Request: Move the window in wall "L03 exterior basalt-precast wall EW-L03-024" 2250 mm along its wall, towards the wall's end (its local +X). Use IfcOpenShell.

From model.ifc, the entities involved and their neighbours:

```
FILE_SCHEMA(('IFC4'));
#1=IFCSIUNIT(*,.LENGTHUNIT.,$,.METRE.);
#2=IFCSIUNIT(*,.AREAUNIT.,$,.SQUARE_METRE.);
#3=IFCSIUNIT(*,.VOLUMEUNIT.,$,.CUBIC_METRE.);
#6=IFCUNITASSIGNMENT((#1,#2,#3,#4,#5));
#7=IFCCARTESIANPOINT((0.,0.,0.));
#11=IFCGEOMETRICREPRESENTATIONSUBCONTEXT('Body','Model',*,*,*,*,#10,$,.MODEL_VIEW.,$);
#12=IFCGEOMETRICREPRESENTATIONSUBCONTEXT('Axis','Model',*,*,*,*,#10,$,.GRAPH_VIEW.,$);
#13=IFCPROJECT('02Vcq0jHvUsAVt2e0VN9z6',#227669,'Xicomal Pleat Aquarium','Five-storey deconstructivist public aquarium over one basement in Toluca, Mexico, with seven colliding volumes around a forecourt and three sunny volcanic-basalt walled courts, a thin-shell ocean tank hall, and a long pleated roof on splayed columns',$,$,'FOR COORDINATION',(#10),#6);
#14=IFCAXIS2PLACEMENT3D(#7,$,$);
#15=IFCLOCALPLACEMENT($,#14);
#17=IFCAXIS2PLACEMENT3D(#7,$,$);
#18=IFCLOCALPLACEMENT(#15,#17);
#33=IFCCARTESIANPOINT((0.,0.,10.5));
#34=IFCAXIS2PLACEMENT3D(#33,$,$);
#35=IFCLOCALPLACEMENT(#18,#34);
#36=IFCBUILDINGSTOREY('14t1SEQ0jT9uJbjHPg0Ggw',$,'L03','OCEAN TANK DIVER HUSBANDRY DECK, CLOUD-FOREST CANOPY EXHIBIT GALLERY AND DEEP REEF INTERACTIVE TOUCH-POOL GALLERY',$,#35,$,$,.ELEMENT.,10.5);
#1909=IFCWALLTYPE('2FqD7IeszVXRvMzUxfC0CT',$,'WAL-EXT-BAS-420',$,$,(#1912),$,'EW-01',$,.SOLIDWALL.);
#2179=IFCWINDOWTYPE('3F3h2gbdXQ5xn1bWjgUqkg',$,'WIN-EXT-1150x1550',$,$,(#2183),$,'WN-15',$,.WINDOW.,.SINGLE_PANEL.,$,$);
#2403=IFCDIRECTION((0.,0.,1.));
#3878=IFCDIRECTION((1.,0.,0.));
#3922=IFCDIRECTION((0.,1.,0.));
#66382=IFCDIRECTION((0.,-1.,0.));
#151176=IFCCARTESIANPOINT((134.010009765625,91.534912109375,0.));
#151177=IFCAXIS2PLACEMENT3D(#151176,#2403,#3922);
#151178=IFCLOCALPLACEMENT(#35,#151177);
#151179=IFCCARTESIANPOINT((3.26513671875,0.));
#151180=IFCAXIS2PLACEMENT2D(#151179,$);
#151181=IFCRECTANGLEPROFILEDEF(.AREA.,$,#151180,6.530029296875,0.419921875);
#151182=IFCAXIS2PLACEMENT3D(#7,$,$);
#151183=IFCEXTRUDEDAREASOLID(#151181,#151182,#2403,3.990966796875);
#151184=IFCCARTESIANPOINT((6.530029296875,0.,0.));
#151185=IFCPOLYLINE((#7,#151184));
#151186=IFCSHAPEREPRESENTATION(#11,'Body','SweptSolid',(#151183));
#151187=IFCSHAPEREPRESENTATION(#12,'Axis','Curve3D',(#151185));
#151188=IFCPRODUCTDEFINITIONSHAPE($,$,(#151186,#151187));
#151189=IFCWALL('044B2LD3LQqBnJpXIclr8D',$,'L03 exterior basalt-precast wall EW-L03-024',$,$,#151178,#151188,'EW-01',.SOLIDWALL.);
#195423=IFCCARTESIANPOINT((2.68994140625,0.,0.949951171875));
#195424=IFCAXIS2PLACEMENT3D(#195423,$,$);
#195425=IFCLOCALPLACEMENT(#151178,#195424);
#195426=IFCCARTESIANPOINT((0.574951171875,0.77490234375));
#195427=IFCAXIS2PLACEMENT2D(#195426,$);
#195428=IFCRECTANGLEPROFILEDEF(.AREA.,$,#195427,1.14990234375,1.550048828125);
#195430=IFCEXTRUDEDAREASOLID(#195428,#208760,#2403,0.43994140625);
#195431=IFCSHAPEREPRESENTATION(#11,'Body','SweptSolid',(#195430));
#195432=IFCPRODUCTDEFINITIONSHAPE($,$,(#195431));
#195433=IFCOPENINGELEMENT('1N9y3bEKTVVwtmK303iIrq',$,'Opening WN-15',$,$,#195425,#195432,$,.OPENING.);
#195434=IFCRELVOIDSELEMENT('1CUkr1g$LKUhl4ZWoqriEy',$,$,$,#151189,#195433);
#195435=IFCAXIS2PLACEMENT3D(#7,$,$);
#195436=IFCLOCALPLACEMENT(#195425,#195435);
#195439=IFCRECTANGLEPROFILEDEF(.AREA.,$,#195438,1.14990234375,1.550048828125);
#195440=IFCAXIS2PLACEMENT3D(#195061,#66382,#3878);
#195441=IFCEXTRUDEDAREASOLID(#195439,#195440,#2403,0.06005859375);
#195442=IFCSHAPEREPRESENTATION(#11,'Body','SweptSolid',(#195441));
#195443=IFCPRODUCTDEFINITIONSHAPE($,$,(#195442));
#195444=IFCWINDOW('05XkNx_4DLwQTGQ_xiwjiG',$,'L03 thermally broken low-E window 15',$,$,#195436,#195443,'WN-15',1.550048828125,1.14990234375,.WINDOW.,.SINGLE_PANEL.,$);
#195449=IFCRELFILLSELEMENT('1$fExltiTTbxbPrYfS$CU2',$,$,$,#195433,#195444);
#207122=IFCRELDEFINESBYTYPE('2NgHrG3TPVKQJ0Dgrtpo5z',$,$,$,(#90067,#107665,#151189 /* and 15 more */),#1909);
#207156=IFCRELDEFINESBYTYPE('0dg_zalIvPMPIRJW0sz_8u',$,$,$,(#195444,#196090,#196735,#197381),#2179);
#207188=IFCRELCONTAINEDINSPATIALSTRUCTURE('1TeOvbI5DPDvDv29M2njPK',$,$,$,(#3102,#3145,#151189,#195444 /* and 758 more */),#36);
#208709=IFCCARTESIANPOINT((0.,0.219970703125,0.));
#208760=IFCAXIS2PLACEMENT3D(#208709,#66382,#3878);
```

```python
import ifcopenshell
import ifcopenshell.api.geometry
import ifcopenshell.util.placement
import ifcopenshell.util.unit

model = ifcopenshell.open("model.ifc")
unit_scale = ifcopenshell.util.unit.calculate_unit_scale(model)

window = model.by_id(195444)
opening = window.FillsVoids[0].RelatingOpeningElement
wall = opening.VoidsElements[0].RelatingBuildingElement

wall_matrix = ifcopenshell.util.placement.get_local_placement(wall.ObjectPlacement)
shift = wall_matrix[:3, 0] * 2.25 / unit_scale
before = ifcopenshell.util.placement.get_local_placement(window.ObjectPlacement)[:3, 3].copy()

# The window is placed relative to its opening, so it follows when the opening moves.
matrix = ifcopenshell.util.placement.get_local_placement(opening.ObjectPlacement)
matrix[:3, 3] += shift
ifcopenshell.api.geometry.edit_object_placement(
    model, product=opening, matrix=matrix, is_si=False, should_transform_children=True
)

after = ifcopenshell.util.placement.get_local_placement(window.ObjectPlacement)[:3, 3]
print("window moved by", (after - before).round(3) + 0.0)

model.write("model_edited.ifc")
```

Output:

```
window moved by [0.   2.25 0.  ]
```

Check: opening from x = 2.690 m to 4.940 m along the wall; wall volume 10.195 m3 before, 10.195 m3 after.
